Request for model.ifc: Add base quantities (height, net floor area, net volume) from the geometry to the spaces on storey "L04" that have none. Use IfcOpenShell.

First a look at what the model holds.

```python
import ifcopenshell
import ifcopenshell.util.element
import ifcopenshell.util.unit

model = ifcopenshell.open("model.ifc")
print(model.schema)
for unit_type in ("LENGTHUNIT", "AREAUNIT", "VOLUMEUNIT"):
    print(unit_type, ifcopenshell.util.unit.calculate_unit_scale(model, unit_type))
storey = next(s for s in model.by_type("IfcBuildingStorey") if s.Name == "L04")
spaces = [e for e in ifcopenshell.util.element.get_decomposition(storey) if e.is_a("IfcSpace")]
for e in sorted(spaces, key=lambda e: e.id()):
    print(e.id(), e.is_a(), e.Name, list(ifcopenshell.util.element.get_psets(e, qtos_only=True)), sep=" | ")
```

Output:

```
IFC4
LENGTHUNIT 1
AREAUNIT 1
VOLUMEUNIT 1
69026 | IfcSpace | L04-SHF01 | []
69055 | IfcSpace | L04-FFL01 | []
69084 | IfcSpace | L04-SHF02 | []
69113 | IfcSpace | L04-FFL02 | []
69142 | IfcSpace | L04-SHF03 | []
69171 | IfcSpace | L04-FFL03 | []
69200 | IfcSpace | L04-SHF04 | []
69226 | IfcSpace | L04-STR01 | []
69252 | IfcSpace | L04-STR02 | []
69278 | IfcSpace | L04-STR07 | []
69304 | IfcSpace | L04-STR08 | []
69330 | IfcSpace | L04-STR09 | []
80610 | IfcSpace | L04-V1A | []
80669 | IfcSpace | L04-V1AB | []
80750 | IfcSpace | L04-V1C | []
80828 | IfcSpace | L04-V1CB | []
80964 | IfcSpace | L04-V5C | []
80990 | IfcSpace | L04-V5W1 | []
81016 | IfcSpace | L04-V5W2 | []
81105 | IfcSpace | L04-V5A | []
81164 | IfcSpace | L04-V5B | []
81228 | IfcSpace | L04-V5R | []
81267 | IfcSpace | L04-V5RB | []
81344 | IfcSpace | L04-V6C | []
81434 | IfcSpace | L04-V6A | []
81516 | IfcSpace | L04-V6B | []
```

```python
import ifcopenshell
import ifcopenshell.api.pset
import ifcopenshell.geom
import ifcopenshell.util.element
import ifcopenshell.util.shape
import ifcopenshell.util.unit

model = ifcopenshell.open("model.ifc")
unit_scale = ifcopenshell.util.unit.calculate_unit_scale(model)
area_scale = ifcopenshell.util.unit.calculate_unit_scale(model, "AREAUNIT")
volume_scale = ifcopenshell.util.unit.calculate_unit_scale(model, "VOLUMEUNIT")
settings = ifcopenshell.geom.settings()

storey = next(s for s in model.by_type("IfcBuildingStorey") if s.Name == "L04")
spaces = [e for e in ifcopenshell.util.element.get_decomposition(storey) if e.is_a("IfcSpace")]

for e in sorted(spaces, key=lambda e: e.id()):
    if ifcopenshell.util.element.get_psets(e, qtos_only=True, should_inherit=False):
        continue
    # Geometry comes back in metres, in the element's own axes.
    shape = ifcopenshell.geom.create_shape(settings, e)
    values = {
        "Height": ifcopenshell.util.shape.get_z(shape.geometry) / unit_scale,
        "NetFloorArea": ifcopenshell.util.shape.get_footprint_area(shape.geometry) / area_scale,
        "NetVolume": ifcopenshell.util.shape.get_volume(shape.geometry) / volume_scale,
    }
    qto = ifcopenshell.api.pset.add_qto(model, product=e, name="Qto_SpaceBaseQuantities")
    ifcopenshell.api.pset.edit_qto(model, qto=qto, properties=values)
    print(e.id(), {k: round(v, 3) for k, v in values.items()})

model.write("model_updated.ifc")
```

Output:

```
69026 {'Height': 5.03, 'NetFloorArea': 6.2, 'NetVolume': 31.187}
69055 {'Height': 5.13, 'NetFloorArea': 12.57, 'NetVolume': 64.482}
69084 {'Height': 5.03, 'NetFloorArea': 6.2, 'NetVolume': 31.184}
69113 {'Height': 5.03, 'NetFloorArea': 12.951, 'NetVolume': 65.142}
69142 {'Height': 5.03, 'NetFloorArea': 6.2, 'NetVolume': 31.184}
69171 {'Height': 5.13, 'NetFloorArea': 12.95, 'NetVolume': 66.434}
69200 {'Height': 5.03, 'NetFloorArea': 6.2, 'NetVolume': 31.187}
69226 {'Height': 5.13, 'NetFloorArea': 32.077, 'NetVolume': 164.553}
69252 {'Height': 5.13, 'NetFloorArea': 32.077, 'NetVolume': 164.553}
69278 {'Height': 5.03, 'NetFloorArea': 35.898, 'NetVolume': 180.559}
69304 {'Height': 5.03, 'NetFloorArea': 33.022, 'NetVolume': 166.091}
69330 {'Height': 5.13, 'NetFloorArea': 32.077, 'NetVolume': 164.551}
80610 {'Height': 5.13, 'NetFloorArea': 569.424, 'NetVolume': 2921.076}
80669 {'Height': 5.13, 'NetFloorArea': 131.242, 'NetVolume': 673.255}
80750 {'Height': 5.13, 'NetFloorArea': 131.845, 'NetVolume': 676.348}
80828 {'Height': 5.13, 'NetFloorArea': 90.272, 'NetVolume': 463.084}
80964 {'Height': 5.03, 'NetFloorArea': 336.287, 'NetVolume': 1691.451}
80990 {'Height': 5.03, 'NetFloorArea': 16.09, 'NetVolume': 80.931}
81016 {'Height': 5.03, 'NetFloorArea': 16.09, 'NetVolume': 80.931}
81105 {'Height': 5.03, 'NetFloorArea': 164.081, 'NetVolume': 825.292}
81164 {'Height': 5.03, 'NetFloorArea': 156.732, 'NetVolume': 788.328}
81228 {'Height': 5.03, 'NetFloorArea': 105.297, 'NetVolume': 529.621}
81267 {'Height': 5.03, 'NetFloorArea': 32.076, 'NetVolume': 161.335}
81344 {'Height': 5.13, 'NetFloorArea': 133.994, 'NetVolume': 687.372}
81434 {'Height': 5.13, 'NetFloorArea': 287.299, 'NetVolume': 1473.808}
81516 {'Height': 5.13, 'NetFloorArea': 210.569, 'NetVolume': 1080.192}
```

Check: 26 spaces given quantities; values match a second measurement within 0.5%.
